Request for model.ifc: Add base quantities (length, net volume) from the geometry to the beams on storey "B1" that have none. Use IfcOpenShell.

First a look at what the model holds.

```python
import ifcopenshell
import ifcopenshell.util.element
import ifcopenshell.util.unit

model = ifcopenshell.open("model.ifc")
print(model.schema)
for unit_type in ("LENGTHUNIT", "AREAUNIT", "VOLUMEUNIT"):
    print(unit_type, ifcopenshell.util.unit.calculate_unit_scale(model, unit_type))
storey = next(s for s in model.by_type("IfcBuildingStorey") if s.Name == "B1")
beams = [e for e in ifcopenshell.util.element.get_decomposition(storey) if e.is_a("IfcBeam")]
for e in sorted(beams, key=lambda e: e.id()):
    print(e.id(), e.is_a(), e.Name, list(ifcopenshell.util.element.get_psets(e, qtos_only=True)), sep=" | ")
```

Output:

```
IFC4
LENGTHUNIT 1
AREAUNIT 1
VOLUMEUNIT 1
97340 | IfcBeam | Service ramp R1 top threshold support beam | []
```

```python
import ifcopenshell
import ifcopenshell.api.pset
import ifcopenshell.geom
import ifcopenshell.util.element
import ifcopenshell.util.shape
import ifcopenshell.util.unit

model = ifcopenshell.open("model.ifc")
unit_scale = ifcopenshell.util.unit.calculate_unit_scale(model)
volume_scale = ifcopenshell.util.unit.calculate_unit_scale(model, "VOLUMEUNIT")
settings = ifcopenshell.geom.settings()

storey = next(s for s in model.by_type("IfcBuildingStorey") if s.Name == "B1")
beams = [e for e in ifcopenshell.util.element.get_decomposition(storey) if e.is_a("IfcBeam")]

for e in sorted(beams, key=lambda e: e.id()):
    if ifcopenshell.util.element.get_psets(e, qtos_only=True, should_inherit=False):
        continue
    # Geometry comes back in metres, in the element's own axes.
    shape = ifcopenshell.geom.create_shape(settings, e)
    values = {
        "Length": ifcopenshell.util.shape.get_max_xyz(shape.geometry) / unit_scale,
        "NetVolume": ifcopenshell.util.shape.get_volume(shape.geometry) / volume_scale,
    }
    qto = ifcopenshell.api.pset.add_qto(model, product=e, name="Qto_BeamBaseQuantities")
    ifcopenshell.api.pset.edit_qto(model, qto=qto, properties=values)
    print(e.id(), {k: round(v, 3) for k, v in values.items()})

model.write("model-out.ifc")
```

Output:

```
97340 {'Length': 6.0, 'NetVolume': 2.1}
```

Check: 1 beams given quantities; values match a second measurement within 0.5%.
